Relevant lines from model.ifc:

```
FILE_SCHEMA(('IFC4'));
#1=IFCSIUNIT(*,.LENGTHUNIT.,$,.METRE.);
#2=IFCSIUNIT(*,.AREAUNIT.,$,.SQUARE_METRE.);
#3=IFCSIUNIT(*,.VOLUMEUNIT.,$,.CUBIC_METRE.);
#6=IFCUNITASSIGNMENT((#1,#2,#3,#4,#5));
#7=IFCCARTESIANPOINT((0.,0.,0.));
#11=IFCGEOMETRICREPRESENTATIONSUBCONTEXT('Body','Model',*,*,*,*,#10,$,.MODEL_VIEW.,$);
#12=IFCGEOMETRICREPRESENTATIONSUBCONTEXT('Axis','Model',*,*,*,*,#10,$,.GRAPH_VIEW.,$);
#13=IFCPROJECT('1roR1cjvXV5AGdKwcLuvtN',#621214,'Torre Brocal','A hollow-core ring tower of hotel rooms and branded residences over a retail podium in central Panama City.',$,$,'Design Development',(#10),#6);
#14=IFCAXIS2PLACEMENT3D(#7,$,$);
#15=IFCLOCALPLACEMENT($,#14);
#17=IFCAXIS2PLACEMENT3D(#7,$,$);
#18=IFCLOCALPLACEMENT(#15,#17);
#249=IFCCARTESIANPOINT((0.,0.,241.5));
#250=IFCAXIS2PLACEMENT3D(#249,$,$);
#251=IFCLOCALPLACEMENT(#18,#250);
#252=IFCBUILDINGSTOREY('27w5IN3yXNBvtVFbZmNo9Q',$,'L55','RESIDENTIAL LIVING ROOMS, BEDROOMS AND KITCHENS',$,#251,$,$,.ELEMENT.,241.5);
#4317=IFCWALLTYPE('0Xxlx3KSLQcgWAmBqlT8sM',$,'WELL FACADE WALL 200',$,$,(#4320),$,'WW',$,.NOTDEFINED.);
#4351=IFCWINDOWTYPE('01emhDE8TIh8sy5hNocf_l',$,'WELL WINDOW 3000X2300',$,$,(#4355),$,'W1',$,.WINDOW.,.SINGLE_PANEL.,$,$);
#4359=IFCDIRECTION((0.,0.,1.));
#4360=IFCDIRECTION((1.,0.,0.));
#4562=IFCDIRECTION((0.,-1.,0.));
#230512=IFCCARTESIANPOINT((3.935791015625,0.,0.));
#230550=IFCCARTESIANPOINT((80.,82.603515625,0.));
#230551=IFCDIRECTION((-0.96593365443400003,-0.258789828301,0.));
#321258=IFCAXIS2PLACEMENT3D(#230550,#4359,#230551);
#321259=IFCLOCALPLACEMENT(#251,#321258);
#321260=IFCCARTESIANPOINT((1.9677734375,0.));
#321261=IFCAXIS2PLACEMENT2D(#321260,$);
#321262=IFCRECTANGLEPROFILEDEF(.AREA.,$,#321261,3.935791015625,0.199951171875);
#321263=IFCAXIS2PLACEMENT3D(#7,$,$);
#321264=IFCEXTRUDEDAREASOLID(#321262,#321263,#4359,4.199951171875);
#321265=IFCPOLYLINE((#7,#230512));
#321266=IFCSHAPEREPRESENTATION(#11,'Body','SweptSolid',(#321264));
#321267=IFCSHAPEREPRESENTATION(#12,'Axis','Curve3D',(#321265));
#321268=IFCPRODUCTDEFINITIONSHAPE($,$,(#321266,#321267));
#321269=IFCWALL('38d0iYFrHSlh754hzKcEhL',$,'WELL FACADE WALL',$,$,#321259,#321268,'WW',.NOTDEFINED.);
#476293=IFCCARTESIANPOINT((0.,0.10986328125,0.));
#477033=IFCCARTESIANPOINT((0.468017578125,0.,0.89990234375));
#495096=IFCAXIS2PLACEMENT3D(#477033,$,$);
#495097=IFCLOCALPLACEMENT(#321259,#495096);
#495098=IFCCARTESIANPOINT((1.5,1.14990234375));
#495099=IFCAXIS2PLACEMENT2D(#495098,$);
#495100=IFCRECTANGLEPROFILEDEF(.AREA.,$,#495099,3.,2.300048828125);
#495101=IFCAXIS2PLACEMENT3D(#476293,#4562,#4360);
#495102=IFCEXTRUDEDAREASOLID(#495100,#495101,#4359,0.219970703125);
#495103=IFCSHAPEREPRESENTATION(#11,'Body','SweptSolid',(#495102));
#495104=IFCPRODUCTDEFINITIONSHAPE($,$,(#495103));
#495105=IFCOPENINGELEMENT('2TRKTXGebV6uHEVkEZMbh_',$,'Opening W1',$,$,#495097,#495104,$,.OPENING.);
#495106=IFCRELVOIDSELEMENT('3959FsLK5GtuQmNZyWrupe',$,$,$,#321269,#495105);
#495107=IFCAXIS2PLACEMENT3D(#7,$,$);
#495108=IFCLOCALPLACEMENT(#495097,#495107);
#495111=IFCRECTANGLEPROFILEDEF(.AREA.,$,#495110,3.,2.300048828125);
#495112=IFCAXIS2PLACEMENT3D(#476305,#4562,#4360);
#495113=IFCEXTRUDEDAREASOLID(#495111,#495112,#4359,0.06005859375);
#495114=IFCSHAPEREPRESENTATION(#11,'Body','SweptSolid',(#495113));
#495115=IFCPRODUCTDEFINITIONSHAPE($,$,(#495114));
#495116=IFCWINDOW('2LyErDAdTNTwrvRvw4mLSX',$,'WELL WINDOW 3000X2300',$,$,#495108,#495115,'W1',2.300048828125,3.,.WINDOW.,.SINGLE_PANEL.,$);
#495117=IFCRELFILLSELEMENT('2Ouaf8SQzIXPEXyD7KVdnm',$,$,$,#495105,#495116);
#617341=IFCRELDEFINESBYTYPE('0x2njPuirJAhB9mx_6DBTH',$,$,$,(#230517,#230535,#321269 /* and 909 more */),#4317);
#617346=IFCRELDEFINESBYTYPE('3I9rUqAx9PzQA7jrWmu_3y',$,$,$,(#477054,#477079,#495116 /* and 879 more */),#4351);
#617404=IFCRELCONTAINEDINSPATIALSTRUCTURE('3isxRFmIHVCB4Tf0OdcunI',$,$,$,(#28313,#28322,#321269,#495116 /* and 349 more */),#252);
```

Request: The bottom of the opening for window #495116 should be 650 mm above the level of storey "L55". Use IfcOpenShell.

```python
import numpy as np
import ifcopenshell
import ifcopenshell.api.geometry
import ifcopenshell.geom
import ifcopenshell.util.element
import ifcopenshell.util.placement
import ifcopenshell.util.shape
import ifcopenshell.util.unit

model = ifcopenshell.open("model.ifc")
unit_scale = ifcopenshell.util.unit.calculate_unit_scale(model)

window = model.by_guid("2LyErDAdTNTwrvRvw4mLSX")
opening = window.FillsVoids[0].RelatingOpeningElement
storey = ifcopenshell.util.element.get_container(window, ifc_class="IfcBuildingStorey")
level = ifcopenshell.util.placement.get_local_placement(storey.ObjectPlacement)[2, 3]

# The opening's origin need not be at the sill, so measure its lowest point.
shape = ifcopenshell.geom.create_shape(ifcopenshell.geom.settings(), opening)
bottom = ifcopenshell.util.shape.get_shape_bottom_elevation(shape, shape.geometry) / unit_scale
dz = level + 0.65 - bottom

shift = np.array([0.0, 0.0, dz])
# The window is placed relative to its opening, so it follows when the opening moves.
matrix = ifcopenshell.util.placement.get_local_placement(opening.ObjectPlacement)
matrix[:3, 3] += shift
ifcopenshell.api.geometry.edit_object_placement(
    model, product=opening, matrix=matrix, is_si=False, should_transform_children=True
)

print(f"moved by {dz * unit_scale:+.3f} m")

model.write("model_edited.ifc")
```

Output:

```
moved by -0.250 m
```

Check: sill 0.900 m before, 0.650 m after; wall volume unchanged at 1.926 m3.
